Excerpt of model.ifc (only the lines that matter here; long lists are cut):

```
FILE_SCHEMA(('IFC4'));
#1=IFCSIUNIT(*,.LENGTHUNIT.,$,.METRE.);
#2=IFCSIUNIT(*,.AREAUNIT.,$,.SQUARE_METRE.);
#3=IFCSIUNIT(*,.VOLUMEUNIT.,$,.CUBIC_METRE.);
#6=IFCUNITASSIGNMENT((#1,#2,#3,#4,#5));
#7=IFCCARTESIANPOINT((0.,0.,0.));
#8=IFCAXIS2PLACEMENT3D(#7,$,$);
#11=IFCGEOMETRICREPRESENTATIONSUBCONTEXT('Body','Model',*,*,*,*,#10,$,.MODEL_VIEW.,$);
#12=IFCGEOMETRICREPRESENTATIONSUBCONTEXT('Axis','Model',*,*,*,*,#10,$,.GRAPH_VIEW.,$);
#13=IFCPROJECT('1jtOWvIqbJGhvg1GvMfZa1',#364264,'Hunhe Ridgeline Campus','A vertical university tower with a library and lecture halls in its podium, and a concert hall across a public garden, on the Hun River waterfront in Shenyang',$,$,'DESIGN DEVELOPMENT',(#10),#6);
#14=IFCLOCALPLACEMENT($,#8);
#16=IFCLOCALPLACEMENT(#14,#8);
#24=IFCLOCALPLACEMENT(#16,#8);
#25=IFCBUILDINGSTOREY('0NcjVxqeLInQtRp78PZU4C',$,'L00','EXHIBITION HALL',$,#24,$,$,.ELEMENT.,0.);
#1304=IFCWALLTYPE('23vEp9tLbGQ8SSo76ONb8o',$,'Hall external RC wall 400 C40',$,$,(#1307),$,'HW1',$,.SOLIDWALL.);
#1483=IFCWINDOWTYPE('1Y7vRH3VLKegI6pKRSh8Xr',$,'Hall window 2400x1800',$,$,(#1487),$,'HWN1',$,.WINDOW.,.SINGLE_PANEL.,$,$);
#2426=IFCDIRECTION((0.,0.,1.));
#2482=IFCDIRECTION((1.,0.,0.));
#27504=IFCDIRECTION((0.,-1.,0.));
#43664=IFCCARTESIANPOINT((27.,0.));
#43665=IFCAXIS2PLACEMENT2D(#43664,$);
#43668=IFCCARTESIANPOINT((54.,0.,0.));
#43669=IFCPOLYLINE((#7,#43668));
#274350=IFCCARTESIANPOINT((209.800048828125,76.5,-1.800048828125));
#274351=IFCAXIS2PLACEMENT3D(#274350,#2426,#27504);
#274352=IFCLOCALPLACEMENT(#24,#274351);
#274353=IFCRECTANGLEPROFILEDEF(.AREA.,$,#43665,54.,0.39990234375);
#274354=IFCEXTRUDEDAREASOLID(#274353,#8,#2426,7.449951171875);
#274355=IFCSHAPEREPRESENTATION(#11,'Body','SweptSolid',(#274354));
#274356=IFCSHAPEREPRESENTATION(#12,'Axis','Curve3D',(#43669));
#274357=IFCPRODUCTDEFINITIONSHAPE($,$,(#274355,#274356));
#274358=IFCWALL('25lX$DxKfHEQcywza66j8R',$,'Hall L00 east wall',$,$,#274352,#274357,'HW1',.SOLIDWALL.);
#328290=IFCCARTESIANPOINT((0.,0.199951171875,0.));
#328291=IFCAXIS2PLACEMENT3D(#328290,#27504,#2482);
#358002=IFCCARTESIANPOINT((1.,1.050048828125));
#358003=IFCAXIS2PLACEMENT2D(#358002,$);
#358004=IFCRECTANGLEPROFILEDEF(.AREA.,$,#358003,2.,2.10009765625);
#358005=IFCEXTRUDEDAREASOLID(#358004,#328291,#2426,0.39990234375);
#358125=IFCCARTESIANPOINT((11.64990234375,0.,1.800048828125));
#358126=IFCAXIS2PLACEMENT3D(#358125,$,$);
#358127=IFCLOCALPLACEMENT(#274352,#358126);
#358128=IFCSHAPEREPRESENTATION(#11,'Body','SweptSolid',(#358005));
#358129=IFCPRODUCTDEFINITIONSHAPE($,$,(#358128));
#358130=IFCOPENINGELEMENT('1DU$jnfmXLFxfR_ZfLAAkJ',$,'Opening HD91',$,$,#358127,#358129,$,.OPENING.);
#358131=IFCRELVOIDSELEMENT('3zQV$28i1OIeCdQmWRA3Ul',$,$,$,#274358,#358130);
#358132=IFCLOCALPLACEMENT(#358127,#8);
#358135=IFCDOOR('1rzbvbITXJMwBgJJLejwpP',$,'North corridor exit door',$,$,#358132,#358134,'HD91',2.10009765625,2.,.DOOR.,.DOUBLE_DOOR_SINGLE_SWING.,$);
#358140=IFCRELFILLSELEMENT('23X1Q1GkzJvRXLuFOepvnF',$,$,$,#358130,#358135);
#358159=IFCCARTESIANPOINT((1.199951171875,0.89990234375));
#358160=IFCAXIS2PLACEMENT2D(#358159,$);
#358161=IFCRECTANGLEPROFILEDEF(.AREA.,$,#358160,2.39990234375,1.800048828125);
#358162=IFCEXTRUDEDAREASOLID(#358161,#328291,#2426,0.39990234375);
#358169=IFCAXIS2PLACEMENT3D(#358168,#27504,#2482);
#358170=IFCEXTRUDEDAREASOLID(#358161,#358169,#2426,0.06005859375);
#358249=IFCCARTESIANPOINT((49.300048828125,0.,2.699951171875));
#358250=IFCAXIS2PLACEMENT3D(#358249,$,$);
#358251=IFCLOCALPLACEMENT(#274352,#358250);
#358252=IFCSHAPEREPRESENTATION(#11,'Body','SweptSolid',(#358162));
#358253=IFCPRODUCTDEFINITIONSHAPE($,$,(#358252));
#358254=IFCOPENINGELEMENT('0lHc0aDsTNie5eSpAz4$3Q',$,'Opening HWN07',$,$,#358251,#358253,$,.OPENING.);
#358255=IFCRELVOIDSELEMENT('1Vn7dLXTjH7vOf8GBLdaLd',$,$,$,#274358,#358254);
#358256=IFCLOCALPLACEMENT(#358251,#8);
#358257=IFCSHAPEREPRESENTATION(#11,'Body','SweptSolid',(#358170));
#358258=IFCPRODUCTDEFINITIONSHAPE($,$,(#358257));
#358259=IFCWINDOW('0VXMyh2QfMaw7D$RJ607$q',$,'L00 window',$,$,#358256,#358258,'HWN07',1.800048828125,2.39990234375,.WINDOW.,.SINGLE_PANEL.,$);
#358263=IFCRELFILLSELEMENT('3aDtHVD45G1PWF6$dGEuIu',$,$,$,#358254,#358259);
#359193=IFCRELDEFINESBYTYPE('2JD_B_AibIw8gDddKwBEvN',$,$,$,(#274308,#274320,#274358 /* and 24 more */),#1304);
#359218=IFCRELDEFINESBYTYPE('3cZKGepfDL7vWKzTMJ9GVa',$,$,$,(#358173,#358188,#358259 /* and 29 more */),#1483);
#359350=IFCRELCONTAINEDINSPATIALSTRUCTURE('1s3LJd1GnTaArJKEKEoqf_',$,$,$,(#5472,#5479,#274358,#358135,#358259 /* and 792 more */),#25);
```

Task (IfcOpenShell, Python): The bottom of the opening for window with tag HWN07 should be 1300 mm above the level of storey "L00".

```python
import numpy as np
import ifcopenshell
import ifcopenshell.api.geometry
import ifcopenshell.geom
import ifcopenshell.util.element
import ifcopenshell.util.placement
import ifcopenshell.util.shape
import ifcopenshell.util.unit

model = ifcopenshell.open("model.ifc")
unit_scale = ifcopenshell.util.unit.calculate_unit_scale(model)

window = model.by_guid("0VXMyh2QfMaw7D$RJ607$q")
opening = window.FillsVoids[0].RelatingOpeningElement
storey = ifcopenshell.util.element.get_container(window, ifc_class="IfcBuildingStorey")
level = ifcopenshell.util.placement.get_local_placement(storey.ObjectPlacement)[2, 3]

# The opening's origin need not be at the sill, so measure its lowest point.
shape = ifcopenshell.geom.create_shape(ifcopenshell.geom.settings(), opening)
bottom = ifcopenshell.util.shape.get_shape_bottom_elevation(shape, shape.geometry) / unit_scale
dz = level + 1.3 / unit_scale - bottom

shift = np.array([0.0, 0.0, dz])
# The window is placed relative to its opening, so it follows when the opening moves.
matrix = ifcopenshell.util.placement.get_local_placement(opening.ObjectPlacement)
matrix[:3, 3] += shift
ifcopenshell.api.geometry.edit_object_placement(
    model, product=opening, matrix=matrix, is_si=False, should_transform_children=True
)

print(f"moved by {dz * unit_scale:+.3f} m")

model.write("model-out.ifc")
```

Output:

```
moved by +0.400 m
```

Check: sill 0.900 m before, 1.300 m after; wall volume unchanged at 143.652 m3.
